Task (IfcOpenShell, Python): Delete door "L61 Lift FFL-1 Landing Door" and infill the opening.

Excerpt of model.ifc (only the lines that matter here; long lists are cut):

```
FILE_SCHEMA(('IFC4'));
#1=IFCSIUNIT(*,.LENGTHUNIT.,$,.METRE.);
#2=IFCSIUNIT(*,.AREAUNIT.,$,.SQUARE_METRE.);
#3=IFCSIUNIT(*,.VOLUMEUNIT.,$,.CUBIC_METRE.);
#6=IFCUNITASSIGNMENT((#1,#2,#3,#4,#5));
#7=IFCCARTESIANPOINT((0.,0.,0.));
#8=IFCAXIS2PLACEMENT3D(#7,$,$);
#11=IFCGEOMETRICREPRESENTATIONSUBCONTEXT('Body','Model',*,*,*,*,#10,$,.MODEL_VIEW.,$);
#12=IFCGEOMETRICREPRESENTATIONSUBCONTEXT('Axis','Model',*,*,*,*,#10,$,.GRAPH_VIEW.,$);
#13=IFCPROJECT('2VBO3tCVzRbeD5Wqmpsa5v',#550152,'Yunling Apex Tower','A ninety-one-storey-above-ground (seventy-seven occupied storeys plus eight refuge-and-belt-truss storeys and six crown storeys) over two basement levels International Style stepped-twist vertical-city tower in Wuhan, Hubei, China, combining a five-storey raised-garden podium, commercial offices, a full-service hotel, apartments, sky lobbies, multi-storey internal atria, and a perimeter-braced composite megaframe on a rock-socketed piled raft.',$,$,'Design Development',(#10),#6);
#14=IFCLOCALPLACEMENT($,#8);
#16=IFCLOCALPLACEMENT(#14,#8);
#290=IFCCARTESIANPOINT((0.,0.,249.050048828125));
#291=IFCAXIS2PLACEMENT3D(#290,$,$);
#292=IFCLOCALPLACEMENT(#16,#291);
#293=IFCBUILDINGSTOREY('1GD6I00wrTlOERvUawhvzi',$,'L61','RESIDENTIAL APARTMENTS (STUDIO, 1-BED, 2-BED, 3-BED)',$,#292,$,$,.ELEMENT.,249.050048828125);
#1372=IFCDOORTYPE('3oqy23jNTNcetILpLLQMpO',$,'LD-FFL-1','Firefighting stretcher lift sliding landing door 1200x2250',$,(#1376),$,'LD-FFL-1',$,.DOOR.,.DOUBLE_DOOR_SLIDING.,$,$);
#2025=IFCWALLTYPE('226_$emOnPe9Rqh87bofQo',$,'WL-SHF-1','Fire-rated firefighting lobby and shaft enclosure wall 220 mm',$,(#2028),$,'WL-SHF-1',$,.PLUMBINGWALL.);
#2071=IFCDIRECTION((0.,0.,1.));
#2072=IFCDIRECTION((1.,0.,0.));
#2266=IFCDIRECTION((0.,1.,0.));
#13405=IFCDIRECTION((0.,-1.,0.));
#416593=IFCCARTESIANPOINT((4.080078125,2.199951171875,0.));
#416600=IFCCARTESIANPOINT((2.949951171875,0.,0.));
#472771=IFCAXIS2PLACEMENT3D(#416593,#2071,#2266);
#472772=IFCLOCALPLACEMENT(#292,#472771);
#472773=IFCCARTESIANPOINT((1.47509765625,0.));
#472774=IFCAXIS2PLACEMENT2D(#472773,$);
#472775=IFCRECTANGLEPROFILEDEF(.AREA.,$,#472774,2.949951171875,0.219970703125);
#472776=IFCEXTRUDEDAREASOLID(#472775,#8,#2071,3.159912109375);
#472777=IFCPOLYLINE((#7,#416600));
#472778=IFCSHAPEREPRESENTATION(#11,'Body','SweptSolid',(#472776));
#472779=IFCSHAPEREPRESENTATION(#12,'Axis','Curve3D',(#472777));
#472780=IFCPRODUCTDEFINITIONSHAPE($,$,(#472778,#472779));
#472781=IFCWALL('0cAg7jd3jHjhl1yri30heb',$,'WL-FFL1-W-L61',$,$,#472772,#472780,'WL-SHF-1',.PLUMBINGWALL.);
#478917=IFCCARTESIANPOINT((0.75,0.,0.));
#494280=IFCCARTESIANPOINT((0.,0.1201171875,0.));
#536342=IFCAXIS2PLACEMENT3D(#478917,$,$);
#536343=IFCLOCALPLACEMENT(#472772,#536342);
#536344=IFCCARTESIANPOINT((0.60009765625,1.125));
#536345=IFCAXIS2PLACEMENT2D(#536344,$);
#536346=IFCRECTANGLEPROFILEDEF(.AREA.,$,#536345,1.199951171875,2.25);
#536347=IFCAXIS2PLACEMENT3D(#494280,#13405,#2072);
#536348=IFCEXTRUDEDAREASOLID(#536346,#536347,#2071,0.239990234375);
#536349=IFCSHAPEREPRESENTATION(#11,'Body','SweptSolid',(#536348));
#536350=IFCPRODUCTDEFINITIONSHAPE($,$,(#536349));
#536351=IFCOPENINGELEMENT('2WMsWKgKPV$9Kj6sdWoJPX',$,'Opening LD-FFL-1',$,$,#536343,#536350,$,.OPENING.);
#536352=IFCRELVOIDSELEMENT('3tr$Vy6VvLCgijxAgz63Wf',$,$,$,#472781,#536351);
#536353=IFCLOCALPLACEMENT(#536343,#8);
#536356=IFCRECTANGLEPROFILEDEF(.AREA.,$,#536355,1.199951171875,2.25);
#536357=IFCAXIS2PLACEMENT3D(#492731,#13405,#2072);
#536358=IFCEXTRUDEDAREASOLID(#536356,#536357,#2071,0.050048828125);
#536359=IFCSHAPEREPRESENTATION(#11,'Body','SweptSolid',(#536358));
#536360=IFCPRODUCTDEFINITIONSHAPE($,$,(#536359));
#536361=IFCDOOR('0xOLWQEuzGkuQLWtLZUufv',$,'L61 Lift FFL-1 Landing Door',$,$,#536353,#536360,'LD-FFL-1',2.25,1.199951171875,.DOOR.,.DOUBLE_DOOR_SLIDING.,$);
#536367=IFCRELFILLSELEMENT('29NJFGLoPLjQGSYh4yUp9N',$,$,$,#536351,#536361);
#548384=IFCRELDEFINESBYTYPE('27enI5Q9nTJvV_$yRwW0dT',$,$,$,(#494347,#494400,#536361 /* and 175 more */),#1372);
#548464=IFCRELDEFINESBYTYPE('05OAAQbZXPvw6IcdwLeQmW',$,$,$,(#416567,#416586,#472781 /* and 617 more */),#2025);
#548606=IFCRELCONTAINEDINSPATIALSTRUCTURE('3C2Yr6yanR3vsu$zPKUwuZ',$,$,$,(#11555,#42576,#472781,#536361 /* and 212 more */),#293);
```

```python
import ifcopenshell
import ifcopenshell.api.feature
import ifcopenshell.api.root
import ifcopenshell.geom
import ifcopenshell.util.shape

model = ifcopenshell.open("model.ifc")
settings = ifcopenshell.geom.settings()


def volume(element):
    """Net volume in cubic metres, openings subtracted."""
    shape = ifcopenshell.geom.create_shape(settings, element)
    return ifcopenshell.util.shape.get_volume(shape.geometry)


door = model.by_guid("0xOLWQEuzGkuQLWtLZUufv")
opening = door.FillsVoids[0].RelatingOpeningElement
wall = opening.VoidsElements[0].RelatingBuildingElement
before = volume(wall)

ifcopenshell.api.root.remove_product(model, product=door)
ifcopenshell.api.feature.remove_feature(model, feature=opening)

after = volume(wall)

print(f"wall volume {before:.3f} -> {after:.3f} m3")

model.write("model_rev.ifc")
```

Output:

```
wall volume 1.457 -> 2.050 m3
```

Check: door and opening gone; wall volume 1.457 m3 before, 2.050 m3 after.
